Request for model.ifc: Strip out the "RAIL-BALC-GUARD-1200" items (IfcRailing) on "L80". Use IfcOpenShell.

First a look at what the model holds.

```python
import ifcopenshell
import ifcopenshell.util.element

model = ifcopenshell.open("model.ifc")
print(model.schema)
storey = next(s for s in model.by_type("IfcBuildingStorey") if s.Name == "L80")
railings = [e for e in ifcopenshell.util.element.get_decomposition(storey) if e.is_a("IfcRailing")]
seen = {}
for e in railings:
    element_type = ifcopenshell.util.element.get_type(e)
    name = element_type.Name if element_type not in (None, e) else None
    seen[name] = seen.get(name, 0) + 1
for name, count in sorted(seen.items(), key=str):
    print(count, "x", name)
```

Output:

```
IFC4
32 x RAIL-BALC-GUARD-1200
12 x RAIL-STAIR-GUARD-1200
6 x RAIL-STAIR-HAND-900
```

```python
import ifcopenshell
import ifcopenshell.api.root
import ifcopenshell.util.element

model = ifcopenshell.open("model.ifc")

storey = next(s for s in model.by_type("IfcBuildingStorey") if s.Name == "L80")
railings = [e for e in ifcopenshell.util.element.get_decomposition(storey) if e.is_a("IfcRailing")]
targets = [e for e in railings if (t := ifcopenshell.util.element.get_type(e)) not in (None, e) and t.Name == "RAIL-BALC-GUARD-1200"]

for e in targets:
    ifcopenshell.api.root.remove_product(model, product=e)
print(len(targets), "removed")

model.write("model-out.ifc")
```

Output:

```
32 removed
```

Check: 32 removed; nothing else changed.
